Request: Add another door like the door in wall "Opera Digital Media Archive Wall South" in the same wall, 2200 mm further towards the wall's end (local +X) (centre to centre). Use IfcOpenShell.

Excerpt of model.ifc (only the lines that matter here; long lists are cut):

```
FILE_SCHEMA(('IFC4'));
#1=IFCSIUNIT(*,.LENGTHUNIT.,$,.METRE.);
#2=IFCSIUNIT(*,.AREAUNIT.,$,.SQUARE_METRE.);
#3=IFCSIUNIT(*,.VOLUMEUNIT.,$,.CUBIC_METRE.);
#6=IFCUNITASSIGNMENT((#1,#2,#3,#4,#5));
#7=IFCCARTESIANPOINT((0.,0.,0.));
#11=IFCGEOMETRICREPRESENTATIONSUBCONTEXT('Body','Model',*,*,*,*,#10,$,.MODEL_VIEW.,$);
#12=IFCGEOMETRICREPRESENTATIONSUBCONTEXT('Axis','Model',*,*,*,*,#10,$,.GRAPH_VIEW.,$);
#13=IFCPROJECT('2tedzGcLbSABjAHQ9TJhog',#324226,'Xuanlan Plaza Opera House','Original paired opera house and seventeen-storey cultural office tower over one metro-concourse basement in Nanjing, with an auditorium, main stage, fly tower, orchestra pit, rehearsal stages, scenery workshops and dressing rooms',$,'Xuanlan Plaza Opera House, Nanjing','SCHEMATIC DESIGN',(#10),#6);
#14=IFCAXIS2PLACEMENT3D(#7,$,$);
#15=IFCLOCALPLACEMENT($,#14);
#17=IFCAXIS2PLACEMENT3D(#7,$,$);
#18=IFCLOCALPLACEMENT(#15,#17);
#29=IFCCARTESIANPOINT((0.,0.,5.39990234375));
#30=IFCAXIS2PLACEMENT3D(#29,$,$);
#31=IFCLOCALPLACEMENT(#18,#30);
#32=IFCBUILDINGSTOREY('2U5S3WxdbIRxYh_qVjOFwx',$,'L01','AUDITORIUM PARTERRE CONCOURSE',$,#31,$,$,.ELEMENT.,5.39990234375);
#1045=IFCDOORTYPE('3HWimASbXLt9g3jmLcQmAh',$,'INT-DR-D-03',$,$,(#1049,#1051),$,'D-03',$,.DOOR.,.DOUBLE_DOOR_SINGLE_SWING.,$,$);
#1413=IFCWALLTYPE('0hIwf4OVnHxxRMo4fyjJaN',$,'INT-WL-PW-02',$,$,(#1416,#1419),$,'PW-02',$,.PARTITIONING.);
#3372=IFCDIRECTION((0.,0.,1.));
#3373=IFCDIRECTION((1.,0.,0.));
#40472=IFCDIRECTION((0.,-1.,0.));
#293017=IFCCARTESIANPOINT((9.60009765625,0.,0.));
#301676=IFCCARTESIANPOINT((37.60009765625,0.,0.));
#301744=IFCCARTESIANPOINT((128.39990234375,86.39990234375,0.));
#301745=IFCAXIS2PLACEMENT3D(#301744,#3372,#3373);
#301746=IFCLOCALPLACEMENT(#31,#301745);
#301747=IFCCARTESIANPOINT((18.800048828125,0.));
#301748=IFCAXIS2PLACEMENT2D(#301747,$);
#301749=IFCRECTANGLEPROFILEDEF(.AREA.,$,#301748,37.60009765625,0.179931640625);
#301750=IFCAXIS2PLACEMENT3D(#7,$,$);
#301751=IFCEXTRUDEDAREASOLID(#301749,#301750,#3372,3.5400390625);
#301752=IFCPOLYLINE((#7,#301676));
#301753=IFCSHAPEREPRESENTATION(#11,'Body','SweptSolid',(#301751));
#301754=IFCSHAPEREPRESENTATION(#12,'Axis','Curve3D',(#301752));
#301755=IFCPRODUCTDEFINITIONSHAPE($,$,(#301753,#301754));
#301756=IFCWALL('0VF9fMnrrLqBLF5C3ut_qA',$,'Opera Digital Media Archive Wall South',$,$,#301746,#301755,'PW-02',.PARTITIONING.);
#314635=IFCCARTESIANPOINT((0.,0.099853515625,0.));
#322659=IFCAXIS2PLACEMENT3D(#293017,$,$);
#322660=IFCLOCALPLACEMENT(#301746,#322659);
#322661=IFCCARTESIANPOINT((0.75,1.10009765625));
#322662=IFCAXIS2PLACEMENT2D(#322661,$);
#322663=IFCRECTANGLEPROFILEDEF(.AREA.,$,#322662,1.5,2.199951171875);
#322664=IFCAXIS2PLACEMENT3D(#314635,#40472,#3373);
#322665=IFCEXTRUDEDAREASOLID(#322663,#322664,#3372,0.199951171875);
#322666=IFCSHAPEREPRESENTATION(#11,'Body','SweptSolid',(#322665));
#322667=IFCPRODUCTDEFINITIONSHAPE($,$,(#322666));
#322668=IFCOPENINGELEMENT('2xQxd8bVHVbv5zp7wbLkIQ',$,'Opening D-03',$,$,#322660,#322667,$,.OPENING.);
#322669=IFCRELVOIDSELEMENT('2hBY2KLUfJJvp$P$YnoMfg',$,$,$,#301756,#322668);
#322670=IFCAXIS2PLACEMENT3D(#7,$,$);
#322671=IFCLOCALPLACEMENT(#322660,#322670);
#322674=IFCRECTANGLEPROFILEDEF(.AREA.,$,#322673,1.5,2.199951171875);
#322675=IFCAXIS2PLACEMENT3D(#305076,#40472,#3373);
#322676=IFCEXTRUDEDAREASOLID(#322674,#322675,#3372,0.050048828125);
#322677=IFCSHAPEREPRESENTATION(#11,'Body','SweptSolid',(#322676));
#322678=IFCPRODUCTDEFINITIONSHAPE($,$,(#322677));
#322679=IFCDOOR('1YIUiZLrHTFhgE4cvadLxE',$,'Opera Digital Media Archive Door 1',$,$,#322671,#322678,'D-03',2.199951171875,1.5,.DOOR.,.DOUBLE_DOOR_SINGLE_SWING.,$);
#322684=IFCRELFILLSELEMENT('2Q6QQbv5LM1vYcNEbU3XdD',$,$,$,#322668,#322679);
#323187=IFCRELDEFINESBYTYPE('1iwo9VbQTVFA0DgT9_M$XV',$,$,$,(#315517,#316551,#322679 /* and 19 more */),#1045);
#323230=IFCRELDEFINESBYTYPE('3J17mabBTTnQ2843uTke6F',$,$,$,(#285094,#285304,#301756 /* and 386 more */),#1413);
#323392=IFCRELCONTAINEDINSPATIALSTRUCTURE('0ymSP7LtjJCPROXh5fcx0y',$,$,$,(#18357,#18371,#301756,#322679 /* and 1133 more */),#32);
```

```python
import ifcopenshell
import ifcopenshell.api.feature
import ifcopenshell.api.geometry
import ifcopenshell.api.root
import ifcopenshell.geom
import ifcopenshell.util.element
import ifcopenshell.util.placement
import ifcopenshell.util.shape
import ifcopenshell.util.unit

model = ifcopenshell.open("model.ifc")
unit_scale = ifcopenshell.util.unit.calculate_unit_scale(model)
settings = ifcopenshell.geom.settings()


def volume(element):
    """Net volume in cubic metres, openings subtracted."""
    shape = ifcopenshell.geom.create_shape(settings, element)
    return ifcopenshell.util.shape.get_volume(shape.geometry)


door = model.by_id(322679)
opening = door.FillsVoids[0].RelatingOpeningElement
wall = opening.VoidsElements[0].RelatingBuildingElement
before = volume(wall)
shift = ifcopenshell.util.placement.get_local_placement(wall.ObjectPlacement)[:3, 0] * 2.2 / unit_scale

# copy_class copies the void relationship, type, container and properties, but no geometry.
new_opening = ifcopenshell.api.root.copy_class(model, product=opening)
new_opening.Representation = ifcopenshell.util.element.copy_deep(
    model, opening.Representation, exclude=["IfcGeometricRepresentationContext", "IfcRepresentationMap"]
)
new_door = ifcopenshell.api.root.copy_class(model, product=door)
new_door.Representation = ifcopenshell.util.element.copy_deep(
    model, door.Representation, exclude=["IfcGeometricRepresentationContext", "IfcRepresentationMap"]
)
new_door.Tag = None
ifcopenshell.api.feature.add_filling(model, opening=new_opening, element=new_door)

for old, new in ((opening, new_opening), (door, new_door)):
    matrix = ifcopenshell.util.placement.get_local_placement(old.ObjectPlacement)
    matrix[:3, 3] += shift
    ifcopenshell.api.geometry.edit_object_placement(model, product=new, matrix=matrix, is_si=False)

after = volume(wall)

print(f"wall volume {before:.3f} -> {after:.3f} m3")

model.write("model_v2.ifc")
```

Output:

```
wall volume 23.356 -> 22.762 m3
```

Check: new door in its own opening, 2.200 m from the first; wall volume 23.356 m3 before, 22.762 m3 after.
